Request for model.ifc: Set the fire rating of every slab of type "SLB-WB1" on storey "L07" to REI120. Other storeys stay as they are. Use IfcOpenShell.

First a look at what the model holds.

```python
import ifcopenshell
import ifcopenshell.util.element

model = ifcopenshell.open("model.ifc")
print(model.schema)
storey = next(s for s in model.by_type("IfcBuildingStorey") if s.Name == "L07")
slabs = [e for e in ifcopenshell.util.element.get_decomposition(storey) if e.is_a("IfcSlab")]
seen = {}
for e in slabs:
    element_type = ifcopenshell.util.element.get_type(e)
    key = (element_type.Name if element_type != e and element_type else None, ifcopenshell.util.element.get_pset(e, "Pset_SlabCommon", "FireRating"))
    seen[key] = seen.get(key, 0) + 1
for (name, value), count in sorted(seen.items(), key=str):
    print(count, "x", name, "|", value)
```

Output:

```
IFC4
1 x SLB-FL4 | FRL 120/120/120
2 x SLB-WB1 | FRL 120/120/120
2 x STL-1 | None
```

```python
import ifcopenshell
import ifcopenshell.api.pset
import ifcopenshell.util.element

model = ifcopenshell.open("model.ifc")

storey = next(s for s in model.by_type("IfcBuildingStorey") if s.Name == "L07")
slabs = [e for e in ifcopenshell.util.element.get_decomposition(storey) if e.is_a("IfcSlab")]

count = 0
for e in slabs:
    element_type = ifcopenshell.util.element.get_type(e)
    if element_type in (None, e) or element_type.Name != "SLB-WB1":
        continue
    found = ifcopenshell.util.element.get_pset(e, "Pset_SlabCommon", should_inherit=False)
    if found:
        pset = model.by_id(found["id"])
        if len(ifcopenshell.util.element.get_elements_by_pset(pset)) > 1:
            pset = ifcopenshell.api.pset.unshare_pset(model, products=[e], pset=pset)[0]
    else:
        pset = ifcopenshell.api.pset.add_pset(model, product=e, name="Pset_SlabCommon")
    ifcopenshell.api.pset.edit_pset(model, pset=pset, properties={"FireRating": "REI120"})
    count += 1

print(count, "slabs updated")

model.write("model-out.ifc")
```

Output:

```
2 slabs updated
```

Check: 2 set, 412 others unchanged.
